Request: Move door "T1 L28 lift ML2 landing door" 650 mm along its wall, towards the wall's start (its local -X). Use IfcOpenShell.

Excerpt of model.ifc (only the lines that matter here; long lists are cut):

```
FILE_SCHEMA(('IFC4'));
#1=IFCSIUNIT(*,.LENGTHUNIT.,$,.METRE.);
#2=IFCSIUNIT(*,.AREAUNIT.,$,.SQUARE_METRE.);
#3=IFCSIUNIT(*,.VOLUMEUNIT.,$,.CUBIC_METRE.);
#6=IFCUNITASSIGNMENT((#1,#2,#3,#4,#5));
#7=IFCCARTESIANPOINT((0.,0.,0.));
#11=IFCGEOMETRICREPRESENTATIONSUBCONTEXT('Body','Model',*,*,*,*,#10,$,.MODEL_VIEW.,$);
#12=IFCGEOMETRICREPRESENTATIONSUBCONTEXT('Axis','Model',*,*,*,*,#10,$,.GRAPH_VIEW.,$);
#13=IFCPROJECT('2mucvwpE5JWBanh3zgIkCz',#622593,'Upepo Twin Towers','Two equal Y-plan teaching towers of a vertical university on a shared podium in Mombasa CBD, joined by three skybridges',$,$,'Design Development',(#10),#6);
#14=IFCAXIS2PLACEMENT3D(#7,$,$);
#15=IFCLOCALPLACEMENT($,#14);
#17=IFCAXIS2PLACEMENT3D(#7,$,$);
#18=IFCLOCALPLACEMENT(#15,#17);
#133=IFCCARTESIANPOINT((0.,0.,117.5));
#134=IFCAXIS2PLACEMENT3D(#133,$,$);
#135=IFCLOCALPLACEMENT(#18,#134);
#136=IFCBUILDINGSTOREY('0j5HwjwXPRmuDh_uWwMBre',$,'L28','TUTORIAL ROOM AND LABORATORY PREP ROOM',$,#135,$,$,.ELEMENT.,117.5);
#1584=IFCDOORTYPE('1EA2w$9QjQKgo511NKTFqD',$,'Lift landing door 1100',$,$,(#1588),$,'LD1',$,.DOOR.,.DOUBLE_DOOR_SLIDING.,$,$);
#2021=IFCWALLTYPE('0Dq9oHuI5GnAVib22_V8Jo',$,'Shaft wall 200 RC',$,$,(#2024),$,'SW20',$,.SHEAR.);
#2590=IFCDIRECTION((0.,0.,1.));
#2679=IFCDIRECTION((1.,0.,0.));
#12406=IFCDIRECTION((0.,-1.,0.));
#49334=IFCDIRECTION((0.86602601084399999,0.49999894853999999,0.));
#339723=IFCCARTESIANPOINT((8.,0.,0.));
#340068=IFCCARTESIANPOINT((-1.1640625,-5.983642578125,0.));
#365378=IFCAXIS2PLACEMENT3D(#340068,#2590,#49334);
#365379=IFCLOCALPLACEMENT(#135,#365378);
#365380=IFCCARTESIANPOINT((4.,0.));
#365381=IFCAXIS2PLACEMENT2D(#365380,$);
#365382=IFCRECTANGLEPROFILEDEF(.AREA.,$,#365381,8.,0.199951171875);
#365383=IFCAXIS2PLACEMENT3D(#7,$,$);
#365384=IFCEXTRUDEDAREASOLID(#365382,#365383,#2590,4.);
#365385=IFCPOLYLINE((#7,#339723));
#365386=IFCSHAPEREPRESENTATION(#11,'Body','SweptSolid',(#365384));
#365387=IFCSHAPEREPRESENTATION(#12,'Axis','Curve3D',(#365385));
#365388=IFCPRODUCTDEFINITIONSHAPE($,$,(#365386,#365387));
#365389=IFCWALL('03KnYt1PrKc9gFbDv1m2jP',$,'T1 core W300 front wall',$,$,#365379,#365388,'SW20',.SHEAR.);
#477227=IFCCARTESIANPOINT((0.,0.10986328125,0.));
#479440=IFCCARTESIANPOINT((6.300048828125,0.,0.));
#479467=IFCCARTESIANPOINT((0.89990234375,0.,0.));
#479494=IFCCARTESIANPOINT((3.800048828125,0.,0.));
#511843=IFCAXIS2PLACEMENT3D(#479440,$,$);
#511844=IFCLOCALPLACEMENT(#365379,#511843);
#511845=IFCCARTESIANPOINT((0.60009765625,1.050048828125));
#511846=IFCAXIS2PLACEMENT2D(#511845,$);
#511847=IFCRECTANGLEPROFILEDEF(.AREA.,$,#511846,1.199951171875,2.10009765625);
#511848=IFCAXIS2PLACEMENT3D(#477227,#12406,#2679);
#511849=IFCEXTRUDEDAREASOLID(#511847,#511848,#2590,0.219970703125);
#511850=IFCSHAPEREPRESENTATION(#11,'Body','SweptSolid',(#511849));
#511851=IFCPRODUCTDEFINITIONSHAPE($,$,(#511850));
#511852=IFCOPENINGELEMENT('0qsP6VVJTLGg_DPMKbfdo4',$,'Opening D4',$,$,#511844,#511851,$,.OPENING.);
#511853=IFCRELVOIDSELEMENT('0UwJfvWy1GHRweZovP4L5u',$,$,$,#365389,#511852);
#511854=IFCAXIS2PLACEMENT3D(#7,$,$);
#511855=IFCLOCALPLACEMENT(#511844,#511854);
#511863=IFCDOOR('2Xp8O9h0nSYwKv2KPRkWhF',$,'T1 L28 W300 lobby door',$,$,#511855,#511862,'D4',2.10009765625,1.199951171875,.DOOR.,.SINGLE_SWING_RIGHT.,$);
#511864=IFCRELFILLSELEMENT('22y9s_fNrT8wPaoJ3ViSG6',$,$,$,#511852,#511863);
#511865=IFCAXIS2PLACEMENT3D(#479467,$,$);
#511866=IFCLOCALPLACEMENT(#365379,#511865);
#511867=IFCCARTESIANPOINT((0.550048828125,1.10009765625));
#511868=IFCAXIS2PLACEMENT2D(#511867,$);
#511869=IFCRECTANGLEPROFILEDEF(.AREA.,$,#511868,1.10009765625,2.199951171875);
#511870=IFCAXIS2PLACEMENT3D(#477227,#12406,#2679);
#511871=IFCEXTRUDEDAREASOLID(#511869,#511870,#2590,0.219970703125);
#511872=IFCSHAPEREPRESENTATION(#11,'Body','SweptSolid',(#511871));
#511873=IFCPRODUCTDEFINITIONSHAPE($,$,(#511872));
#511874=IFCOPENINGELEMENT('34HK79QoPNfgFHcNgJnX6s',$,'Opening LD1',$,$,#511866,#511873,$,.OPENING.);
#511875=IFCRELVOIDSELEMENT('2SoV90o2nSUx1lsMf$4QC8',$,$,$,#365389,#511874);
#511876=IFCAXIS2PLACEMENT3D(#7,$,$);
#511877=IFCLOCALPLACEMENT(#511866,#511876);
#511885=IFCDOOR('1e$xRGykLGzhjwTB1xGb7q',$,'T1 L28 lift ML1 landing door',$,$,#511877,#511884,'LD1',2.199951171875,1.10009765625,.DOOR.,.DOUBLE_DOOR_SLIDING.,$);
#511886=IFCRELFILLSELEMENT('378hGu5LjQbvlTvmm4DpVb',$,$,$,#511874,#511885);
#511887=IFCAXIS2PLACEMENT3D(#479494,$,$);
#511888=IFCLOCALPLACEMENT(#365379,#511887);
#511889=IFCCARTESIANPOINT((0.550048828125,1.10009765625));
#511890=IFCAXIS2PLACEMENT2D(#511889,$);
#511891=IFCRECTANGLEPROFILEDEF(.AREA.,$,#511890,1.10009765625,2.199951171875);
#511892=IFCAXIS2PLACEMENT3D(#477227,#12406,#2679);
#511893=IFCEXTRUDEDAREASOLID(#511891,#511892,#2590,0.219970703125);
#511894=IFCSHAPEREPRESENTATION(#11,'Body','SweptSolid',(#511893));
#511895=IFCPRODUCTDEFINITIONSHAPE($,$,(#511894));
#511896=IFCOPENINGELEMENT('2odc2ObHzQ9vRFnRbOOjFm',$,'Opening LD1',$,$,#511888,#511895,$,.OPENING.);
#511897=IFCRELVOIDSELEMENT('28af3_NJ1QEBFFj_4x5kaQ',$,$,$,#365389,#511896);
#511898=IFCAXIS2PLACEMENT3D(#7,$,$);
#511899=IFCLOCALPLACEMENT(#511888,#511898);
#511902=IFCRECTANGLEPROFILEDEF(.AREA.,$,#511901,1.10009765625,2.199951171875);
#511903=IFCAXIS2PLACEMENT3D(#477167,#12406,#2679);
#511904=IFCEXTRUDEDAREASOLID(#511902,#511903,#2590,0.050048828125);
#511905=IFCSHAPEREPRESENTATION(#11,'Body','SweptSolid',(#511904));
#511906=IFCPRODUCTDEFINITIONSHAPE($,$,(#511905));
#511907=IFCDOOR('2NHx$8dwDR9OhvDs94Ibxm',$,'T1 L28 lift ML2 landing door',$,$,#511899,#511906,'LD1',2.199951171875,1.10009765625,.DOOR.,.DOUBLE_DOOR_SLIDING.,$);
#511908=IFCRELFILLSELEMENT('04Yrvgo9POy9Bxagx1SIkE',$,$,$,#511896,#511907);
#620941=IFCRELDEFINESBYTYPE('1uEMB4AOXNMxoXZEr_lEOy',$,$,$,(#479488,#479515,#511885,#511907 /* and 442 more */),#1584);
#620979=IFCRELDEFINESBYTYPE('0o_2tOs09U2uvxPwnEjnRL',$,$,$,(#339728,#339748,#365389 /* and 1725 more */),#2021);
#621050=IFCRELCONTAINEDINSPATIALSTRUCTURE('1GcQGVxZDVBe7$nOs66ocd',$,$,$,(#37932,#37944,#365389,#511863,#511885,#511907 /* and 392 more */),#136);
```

```python
import ifcopenshell
import ifcopenshell.api.geometry
import ifcopenshell.util.placement
import ifcopenshell.util.unit

model = ifcopenshell.open("model.ifc")
unit_scale = ifcopenshell.util.unit.calculate_unit_scale(model)

door = model.by_id(511907)
opening = door.FillsVoids[0].RelatingOpeningElement
wall = opening.VoidsElements[0].RelatingBuildingElement

wall_matrix = ifcopenshell.util.placement.get_local_placement(wall.ObjectPlacement)
shift = wall_matrix[:3, 0] * -0.65 / unit_scale
before = ifcopenshell.util.placement.get_local_placement(door.ObjectPlacement)[:3, 3].copy()

# The door is placed relative to its opening, so it follows when the opening moves.
matrix = ifcopenshell.util.placement.get_local_placement(opening.ObjectPlacement)
matrix[:3, 3] += shift
ifcopenshell.api.geometry.edit_object_placement(
    model, product=opening, matrix=matrix, is_si=False, should_transform_children=True
)

after = ifcopenshell.util.placement.get_local_placement(door.ObjectPlacement)[:3, 3]
print("door moved by", (after - before).round(3) + 0.0)

model.write("model_edited.ifc")
```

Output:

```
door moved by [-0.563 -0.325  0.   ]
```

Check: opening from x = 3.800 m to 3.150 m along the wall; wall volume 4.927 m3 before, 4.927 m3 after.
